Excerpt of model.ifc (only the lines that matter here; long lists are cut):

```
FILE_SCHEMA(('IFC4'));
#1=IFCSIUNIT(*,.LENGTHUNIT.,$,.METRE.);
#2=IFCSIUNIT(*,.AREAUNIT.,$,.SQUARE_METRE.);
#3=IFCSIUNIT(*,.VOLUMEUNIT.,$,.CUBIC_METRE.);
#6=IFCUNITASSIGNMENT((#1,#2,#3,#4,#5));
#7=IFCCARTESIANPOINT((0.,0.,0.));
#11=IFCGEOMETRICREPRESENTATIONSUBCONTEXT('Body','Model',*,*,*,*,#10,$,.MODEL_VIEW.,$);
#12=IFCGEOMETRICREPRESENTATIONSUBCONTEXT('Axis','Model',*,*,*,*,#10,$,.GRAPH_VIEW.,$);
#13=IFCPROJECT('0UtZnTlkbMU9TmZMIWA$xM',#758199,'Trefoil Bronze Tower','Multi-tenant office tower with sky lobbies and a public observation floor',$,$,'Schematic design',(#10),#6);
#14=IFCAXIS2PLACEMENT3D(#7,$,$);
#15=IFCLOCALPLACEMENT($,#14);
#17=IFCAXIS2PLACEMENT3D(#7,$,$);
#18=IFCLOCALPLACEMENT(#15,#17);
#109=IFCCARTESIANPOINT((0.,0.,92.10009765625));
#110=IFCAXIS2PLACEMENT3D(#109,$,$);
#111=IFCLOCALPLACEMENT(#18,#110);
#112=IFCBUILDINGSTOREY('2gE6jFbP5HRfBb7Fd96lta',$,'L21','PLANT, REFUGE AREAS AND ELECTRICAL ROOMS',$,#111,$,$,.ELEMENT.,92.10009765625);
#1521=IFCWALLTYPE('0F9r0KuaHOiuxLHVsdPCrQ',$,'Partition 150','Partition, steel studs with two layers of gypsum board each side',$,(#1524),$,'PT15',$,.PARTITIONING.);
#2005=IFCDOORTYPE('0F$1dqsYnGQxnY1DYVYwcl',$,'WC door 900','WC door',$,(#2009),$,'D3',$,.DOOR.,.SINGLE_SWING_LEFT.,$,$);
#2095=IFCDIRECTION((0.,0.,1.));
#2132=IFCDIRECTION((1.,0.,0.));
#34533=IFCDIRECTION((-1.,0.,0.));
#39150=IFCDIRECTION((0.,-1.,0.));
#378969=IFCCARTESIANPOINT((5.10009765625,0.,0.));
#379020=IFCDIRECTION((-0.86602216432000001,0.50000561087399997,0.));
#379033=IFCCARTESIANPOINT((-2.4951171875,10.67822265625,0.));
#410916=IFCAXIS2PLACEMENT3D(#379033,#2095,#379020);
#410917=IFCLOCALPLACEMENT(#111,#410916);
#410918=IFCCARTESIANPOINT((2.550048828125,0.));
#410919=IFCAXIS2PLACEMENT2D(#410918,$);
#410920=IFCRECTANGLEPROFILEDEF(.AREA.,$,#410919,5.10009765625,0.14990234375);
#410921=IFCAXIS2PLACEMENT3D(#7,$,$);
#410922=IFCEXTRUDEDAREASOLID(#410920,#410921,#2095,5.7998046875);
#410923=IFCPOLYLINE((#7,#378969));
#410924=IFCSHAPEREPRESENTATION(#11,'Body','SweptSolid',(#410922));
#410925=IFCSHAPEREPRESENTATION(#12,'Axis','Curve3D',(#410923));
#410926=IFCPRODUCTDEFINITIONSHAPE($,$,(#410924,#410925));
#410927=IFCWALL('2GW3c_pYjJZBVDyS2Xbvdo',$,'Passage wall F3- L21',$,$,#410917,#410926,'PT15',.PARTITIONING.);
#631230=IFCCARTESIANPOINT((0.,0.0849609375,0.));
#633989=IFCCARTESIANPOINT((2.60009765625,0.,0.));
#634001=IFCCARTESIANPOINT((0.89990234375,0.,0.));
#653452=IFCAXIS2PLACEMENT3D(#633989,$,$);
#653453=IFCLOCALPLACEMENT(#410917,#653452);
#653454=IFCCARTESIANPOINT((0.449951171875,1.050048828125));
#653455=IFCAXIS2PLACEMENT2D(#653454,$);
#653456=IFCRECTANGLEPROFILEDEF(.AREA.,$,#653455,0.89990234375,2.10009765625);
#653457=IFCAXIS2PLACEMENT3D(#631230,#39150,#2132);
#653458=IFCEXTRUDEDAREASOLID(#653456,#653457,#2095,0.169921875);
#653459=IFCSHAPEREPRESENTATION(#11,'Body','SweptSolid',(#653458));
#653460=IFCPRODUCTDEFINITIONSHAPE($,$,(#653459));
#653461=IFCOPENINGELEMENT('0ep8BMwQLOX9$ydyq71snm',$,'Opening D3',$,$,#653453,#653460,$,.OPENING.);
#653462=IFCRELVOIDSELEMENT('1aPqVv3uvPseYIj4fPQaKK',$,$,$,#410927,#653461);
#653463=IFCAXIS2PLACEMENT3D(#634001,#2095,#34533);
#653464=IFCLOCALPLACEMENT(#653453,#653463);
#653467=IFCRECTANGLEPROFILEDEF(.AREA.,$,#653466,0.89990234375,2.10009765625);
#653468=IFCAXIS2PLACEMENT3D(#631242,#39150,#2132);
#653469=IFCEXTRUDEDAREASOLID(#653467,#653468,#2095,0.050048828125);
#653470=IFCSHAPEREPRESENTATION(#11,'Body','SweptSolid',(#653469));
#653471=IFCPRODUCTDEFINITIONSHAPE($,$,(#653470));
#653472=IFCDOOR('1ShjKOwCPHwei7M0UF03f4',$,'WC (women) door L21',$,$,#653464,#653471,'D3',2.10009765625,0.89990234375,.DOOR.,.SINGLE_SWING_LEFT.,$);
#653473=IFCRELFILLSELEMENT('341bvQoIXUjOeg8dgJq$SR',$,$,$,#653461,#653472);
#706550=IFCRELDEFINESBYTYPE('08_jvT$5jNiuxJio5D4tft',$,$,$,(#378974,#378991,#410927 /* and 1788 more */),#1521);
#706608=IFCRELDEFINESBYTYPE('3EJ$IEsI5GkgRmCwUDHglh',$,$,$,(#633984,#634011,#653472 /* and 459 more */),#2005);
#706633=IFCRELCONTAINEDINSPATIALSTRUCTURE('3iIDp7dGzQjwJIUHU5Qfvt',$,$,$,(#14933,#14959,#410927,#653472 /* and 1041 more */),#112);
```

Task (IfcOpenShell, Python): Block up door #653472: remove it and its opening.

```python
import ifcopenshell
import ifcopenshell.api.feature
import ifcopenshell.api.root
import ifcopenshell.geom
import ifcopenshell.util.shape

model = ifcopenshell.open("model.ifc")
settings = ifcopenshell.geom.settings()


def volume(element):
    """Net volume in cubic metres, openings subtracted."""
    shape = ifcopenshell.geom.create_shape(settings, element)
    return ifcopenshell.util.shape.get_volume(shape.geometry)


door = model.by_id(653472)
opening = door.FillsVoids[0].RelatingOpeningElement
wall = opening.VoidsElements[0].RelatingBuildingElement
before = volume(wall)

ifcopenshell.api.root.remove_product(model, product=door)
ifcopenshell.api.feature.remove_feature(model, feature=opening)

after = volume(wall)

print(f"wall volume {before:.3f} -> {after:.3f} m3")

model.write("model-out.ifc")
```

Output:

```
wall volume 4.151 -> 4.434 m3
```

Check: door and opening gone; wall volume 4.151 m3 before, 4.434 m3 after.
